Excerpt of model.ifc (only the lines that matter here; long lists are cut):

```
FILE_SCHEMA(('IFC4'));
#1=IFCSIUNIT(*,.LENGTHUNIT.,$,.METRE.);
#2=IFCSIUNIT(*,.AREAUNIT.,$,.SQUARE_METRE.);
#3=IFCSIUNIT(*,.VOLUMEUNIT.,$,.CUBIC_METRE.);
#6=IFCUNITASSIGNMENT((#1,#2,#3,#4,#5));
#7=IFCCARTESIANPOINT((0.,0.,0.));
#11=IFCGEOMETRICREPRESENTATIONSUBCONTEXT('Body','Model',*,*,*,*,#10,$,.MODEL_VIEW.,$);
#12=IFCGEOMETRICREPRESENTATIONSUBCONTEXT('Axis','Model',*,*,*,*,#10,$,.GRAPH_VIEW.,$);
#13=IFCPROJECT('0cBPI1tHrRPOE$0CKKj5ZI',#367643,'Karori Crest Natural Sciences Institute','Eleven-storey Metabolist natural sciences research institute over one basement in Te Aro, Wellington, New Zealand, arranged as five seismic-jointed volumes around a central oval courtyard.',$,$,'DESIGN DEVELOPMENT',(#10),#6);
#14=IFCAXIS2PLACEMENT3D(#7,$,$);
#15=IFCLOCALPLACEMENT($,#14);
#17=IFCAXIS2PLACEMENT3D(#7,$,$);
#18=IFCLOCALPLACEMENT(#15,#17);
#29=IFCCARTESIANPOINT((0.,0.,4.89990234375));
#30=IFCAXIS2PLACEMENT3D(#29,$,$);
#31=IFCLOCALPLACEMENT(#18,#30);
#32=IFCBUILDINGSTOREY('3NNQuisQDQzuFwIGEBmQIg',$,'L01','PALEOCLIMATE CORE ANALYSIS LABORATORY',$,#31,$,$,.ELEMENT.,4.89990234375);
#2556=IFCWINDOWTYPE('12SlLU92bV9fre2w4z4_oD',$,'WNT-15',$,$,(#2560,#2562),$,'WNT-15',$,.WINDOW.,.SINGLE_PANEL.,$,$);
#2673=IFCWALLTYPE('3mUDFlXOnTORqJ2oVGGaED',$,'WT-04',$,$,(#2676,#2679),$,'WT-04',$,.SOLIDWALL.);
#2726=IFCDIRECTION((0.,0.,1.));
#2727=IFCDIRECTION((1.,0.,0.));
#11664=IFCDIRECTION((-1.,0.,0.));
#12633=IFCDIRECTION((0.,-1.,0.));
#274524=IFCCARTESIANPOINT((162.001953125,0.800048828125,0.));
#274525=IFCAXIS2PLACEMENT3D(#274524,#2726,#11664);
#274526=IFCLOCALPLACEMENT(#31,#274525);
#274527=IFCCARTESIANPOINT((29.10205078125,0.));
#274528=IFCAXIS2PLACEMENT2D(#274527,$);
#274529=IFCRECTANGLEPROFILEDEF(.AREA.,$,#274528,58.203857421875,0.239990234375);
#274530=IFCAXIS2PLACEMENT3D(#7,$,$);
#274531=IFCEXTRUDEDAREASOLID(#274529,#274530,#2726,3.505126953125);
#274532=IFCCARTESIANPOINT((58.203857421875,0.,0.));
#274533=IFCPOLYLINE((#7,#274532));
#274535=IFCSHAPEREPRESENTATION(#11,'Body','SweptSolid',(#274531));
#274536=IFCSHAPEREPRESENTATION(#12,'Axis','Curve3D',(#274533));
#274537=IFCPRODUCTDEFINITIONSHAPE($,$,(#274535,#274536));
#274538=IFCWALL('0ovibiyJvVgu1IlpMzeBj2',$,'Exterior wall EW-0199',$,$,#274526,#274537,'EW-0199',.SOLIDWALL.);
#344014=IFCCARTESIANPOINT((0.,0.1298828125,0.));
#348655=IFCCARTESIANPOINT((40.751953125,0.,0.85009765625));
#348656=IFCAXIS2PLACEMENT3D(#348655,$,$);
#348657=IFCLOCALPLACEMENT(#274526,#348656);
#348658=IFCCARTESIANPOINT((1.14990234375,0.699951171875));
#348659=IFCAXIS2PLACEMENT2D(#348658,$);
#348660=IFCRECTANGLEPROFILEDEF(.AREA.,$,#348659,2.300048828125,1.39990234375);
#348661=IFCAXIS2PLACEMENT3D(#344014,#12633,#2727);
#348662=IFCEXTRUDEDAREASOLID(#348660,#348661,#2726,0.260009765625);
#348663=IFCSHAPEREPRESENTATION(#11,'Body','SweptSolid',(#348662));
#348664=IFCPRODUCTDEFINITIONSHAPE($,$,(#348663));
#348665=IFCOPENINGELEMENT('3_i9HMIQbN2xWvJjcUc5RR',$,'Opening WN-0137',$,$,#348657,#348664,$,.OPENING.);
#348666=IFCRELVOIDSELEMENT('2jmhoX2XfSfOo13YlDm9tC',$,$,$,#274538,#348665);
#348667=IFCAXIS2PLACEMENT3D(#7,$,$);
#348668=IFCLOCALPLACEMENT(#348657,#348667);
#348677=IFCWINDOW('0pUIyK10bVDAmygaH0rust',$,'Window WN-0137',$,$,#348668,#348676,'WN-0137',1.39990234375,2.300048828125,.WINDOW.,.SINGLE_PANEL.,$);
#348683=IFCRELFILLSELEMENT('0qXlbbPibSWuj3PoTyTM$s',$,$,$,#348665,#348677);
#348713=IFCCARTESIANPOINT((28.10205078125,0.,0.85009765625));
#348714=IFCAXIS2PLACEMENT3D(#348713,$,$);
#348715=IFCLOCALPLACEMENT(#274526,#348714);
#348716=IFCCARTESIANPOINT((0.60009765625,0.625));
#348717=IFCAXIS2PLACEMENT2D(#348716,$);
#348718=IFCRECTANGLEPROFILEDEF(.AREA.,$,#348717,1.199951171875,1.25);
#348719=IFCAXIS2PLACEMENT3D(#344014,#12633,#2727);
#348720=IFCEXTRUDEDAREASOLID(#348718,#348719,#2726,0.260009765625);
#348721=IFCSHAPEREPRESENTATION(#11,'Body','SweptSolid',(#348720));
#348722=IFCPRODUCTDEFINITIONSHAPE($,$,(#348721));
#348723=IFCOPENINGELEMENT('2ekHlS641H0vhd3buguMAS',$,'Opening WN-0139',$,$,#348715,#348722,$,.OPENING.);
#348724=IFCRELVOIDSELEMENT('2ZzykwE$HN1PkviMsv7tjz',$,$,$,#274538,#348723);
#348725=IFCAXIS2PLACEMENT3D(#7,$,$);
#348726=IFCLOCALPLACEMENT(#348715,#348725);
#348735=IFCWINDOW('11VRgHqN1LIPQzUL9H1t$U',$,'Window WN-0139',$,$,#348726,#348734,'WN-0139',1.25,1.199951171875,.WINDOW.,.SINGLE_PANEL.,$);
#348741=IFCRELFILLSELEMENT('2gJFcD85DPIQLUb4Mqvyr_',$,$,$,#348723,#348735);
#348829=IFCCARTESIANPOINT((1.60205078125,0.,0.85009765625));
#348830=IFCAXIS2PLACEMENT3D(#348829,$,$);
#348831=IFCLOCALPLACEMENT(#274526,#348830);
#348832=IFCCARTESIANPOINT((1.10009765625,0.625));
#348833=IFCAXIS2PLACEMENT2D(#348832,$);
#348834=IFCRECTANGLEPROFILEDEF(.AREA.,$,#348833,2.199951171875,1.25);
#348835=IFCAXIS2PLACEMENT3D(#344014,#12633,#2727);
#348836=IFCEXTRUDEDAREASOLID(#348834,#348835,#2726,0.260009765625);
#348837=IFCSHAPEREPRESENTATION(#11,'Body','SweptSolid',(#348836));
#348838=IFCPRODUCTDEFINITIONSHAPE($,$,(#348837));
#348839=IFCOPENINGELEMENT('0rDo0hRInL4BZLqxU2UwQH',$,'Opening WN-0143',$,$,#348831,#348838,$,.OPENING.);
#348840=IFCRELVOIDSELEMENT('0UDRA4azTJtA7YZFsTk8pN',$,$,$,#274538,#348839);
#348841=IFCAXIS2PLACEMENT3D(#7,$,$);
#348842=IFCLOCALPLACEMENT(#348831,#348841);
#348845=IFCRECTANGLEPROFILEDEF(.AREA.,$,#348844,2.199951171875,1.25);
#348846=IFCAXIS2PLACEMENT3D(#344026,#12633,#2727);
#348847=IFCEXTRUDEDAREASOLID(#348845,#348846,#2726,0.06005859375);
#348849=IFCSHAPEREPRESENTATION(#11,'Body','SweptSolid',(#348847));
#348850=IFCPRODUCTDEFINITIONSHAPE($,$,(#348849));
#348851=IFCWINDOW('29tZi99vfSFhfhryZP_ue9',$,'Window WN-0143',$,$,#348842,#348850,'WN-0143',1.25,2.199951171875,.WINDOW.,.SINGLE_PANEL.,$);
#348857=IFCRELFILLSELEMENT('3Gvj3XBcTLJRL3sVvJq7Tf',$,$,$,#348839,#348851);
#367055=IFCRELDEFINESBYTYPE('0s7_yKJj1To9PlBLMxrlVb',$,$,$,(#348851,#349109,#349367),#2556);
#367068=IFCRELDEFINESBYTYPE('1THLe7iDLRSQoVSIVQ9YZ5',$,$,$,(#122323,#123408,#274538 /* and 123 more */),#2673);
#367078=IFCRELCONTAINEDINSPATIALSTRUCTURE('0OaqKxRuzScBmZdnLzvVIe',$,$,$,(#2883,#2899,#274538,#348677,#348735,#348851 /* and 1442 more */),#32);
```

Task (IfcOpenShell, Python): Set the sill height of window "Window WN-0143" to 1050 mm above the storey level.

```python
import numpy as np
import ifcopenshell
import ifcopenshell.api.geometry
import ifcopenshell.geom
import ifcopenshell.util.element
import ifcopenshell.util.placement
import ifcopenshell.util.shape
import ifcopenshell.util.unit

model = ifcopenshell.open("model.ifc")
unit_scale = ifcopenshell.util.unit.calculate_unit_scale(model)

window = model.by_id(348851)
opening = window.FillsVoids[0].RelatingOpeningElement
storey = ifcopenshell.util.element.get_container(window, ifc_class="IfcBuildingStorey")
level = ifcopenshell.util.placement.get_local_placement(storey.ObjectPlacement)[2, 3]

# The opening's origin need not be at the sill, so measure its lowest point.
shape = ifcopenshell.geom.create_shape(ifcopenshell.geom.settings(), opening)
bottom = ifcopenshell.util.shape.get_shape_bottom_elevation(shape, shape.geometry) / unit_scale
dz = level + 1.05 - bottom

shift = np.array([0.0, 0.0, dz])
# The window is placed relative to its opening, so it follows when the opening moves.
matrix = ifcopenshell.util.placement.get_local_placement(opening.ObjectPlacement)
matrix[:3, 3] += shift
ifcopenshell.api.geometry.edit_object_placement(
    model, product=opening, matrix=matrix, is_si=False, should_transform_children=True
)

print(f"moved by {dz * unit_scale:+.3f} m")

model.write("model_v2.ifc")
```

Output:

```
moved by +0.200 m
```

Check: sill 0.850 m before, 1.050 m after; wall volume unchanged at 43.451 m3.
